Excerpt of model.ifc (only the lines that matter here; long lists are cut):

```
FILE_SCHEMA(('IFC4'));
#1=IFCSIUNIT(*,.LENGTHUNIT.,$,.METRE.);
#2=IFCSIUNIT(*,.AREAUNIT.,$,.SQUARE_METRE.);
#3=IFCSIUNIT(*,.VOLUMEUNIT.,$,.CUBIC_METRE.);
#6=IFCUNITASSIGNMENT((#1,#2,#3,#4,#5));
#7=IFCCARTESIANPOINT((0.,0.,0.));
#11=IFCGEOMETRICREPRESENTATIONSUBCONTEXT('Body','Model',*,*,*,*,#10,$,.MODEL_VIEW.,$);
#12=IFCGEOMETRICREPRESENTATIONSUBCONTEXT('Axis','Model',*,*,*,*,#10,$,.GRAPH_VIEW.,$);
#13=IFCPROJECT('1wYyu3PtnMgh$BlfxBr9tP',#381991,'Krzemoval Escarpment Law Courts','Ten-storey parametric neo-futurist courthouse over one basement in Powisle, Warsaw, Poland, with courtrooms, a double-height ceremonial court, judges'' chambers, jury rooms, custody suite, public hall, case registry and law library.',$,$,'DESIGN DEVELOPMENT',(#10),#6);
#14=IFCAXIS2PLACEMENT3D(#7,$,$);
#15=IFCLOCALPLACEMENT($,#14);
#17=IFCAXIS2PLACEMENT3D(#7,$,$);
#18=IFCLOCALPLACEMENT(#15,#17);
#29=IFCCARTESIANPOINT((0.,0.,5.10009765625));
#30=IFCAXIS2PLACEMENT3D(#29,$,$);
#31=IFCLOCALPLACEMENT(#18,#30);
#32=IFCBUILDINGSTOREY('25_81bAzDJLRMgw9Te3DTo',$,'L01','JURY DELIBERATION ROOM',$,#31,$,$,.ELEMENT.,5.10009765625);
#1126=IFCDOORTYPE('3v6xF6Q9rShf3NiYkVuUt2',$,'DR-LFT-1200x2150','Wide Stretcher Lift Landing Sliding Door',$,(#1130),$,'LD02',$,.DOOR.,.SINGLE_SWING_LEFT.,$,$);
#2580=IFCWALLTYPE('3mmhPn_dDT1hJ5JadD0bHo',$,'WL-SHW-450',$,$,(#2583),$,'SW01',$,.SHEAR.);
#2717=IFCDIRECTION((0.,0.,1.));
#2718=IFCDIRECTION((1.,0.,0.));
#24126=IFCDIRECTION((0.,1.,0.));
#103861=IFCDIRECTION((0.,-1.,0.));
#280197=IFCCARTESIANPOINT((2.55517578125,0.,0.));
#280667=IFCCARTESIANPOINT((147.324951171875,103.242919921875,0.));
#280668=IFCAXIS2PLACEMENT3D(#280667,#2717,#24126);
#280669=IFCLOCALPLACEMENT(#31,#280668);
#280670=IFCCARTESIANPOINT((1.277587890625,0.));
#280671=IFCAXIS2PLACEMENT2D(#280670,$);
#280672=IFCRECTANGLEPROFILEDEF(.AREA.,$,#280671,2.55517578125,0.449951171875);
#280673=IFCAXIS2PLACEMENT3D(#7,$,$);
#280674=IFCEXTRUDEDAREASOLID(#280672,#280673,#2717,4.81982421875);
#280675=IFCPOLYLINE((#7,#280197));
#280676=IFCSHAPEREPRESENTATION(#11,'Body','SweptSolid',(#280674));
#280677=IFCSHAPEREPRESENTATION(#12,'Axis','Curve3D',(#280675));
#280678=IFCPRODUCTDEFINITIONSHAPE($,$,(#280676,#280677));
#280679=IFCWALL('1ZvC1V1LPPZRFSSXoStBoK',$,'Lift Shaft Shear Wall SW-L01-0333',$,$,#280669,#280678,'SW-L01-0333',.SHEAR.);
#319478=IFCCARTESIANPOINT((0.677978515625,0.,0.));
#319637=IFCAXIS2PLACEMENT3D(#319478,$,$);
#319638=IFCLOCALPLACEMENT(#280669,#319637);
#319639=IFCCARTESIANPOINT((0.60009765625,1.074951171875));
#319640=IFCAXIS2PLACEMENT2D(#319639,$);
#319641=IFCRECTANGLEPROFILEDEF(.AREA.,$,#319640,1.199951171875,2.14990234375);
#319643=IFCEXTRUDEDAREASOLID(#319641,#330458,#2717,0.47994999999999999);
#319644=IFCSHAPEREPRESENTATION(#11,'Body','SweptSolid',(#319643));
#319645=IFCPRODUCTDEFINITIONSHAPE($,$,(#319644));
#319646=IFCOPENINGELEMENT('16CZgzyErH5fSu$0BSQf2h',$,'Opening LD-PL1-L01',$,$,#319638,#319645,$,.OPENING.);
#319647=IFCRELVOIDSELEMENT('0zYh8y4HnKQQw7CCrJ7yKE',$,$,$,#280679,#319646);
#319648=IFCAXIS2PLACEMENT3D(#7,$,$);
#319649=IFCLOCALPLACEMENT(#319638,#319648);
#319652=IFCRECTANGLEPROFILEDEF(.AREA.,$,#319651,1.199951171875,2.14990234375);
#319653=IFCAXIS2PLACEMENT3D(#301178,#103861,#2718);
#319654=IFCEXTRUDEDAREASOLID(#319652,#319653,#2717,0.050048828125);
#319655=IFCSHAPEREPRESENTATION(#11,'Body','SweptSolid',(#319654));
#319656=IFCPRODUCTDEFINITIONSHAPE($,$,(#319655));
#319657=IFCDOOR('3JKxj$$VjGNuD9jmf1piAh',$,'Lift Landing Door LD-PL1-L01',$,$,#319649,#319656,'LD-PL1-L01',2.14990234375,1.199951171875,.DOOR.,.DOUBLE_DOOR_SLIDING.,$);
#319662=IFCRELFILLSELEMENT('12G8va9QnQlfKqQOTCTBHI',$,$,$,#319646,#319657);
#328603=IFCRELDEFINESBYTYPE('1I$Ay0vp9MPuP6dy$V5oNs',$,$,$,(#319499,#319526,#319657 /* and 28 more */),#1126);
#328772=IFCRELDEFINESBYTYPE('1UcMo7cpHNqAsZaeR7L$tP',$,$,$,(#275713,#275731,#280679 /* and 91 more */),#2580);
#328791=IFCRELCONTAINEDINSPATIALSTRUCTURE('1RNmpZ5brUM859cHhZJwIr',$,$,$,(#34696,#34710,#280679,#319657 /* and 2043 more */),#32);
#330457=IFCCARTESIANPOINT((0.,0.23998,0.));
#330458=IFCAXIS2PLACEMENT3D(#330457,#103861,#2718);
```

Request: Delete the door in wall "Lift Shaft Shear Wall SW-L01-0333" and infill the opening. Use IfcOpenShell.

```python
import ifcopenshell
import ifcopenshell.api.feature
import ifcopenshell.api.root
import ifcopenshell.geom
import ifcopenshell.util.shape

model = ifcopenshell.open("model.ifc")
settings = ifcopenshell.geom.settings()


def volume(element):
    """Net volume in cubic metres, openings subtracted."""
    shape = ifcopenshell.geom.create_shape(settings, element)
    return ifcopenshell.util.shape.get_volume(shape.geometry)


door = model.by_id(319657)
opening = door.FillsVoids[0].RelatingOpeningElement
wall = opening.VoidsElements[0].RelatingBuildingElement
before = volume(wall)

ifcopenshell.api.root.remove_product(model, product=door)
ifcopenshell.api.feature.remove_feature(model, feature=opening)

after = volume(wall)

print(f"wall volume {before:.3f} -> {after:.3f} m3")

model.write("model_updated.ifc")
```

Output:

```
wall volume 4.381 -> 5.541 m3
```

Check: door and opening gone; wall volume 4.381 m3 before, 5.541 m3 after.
